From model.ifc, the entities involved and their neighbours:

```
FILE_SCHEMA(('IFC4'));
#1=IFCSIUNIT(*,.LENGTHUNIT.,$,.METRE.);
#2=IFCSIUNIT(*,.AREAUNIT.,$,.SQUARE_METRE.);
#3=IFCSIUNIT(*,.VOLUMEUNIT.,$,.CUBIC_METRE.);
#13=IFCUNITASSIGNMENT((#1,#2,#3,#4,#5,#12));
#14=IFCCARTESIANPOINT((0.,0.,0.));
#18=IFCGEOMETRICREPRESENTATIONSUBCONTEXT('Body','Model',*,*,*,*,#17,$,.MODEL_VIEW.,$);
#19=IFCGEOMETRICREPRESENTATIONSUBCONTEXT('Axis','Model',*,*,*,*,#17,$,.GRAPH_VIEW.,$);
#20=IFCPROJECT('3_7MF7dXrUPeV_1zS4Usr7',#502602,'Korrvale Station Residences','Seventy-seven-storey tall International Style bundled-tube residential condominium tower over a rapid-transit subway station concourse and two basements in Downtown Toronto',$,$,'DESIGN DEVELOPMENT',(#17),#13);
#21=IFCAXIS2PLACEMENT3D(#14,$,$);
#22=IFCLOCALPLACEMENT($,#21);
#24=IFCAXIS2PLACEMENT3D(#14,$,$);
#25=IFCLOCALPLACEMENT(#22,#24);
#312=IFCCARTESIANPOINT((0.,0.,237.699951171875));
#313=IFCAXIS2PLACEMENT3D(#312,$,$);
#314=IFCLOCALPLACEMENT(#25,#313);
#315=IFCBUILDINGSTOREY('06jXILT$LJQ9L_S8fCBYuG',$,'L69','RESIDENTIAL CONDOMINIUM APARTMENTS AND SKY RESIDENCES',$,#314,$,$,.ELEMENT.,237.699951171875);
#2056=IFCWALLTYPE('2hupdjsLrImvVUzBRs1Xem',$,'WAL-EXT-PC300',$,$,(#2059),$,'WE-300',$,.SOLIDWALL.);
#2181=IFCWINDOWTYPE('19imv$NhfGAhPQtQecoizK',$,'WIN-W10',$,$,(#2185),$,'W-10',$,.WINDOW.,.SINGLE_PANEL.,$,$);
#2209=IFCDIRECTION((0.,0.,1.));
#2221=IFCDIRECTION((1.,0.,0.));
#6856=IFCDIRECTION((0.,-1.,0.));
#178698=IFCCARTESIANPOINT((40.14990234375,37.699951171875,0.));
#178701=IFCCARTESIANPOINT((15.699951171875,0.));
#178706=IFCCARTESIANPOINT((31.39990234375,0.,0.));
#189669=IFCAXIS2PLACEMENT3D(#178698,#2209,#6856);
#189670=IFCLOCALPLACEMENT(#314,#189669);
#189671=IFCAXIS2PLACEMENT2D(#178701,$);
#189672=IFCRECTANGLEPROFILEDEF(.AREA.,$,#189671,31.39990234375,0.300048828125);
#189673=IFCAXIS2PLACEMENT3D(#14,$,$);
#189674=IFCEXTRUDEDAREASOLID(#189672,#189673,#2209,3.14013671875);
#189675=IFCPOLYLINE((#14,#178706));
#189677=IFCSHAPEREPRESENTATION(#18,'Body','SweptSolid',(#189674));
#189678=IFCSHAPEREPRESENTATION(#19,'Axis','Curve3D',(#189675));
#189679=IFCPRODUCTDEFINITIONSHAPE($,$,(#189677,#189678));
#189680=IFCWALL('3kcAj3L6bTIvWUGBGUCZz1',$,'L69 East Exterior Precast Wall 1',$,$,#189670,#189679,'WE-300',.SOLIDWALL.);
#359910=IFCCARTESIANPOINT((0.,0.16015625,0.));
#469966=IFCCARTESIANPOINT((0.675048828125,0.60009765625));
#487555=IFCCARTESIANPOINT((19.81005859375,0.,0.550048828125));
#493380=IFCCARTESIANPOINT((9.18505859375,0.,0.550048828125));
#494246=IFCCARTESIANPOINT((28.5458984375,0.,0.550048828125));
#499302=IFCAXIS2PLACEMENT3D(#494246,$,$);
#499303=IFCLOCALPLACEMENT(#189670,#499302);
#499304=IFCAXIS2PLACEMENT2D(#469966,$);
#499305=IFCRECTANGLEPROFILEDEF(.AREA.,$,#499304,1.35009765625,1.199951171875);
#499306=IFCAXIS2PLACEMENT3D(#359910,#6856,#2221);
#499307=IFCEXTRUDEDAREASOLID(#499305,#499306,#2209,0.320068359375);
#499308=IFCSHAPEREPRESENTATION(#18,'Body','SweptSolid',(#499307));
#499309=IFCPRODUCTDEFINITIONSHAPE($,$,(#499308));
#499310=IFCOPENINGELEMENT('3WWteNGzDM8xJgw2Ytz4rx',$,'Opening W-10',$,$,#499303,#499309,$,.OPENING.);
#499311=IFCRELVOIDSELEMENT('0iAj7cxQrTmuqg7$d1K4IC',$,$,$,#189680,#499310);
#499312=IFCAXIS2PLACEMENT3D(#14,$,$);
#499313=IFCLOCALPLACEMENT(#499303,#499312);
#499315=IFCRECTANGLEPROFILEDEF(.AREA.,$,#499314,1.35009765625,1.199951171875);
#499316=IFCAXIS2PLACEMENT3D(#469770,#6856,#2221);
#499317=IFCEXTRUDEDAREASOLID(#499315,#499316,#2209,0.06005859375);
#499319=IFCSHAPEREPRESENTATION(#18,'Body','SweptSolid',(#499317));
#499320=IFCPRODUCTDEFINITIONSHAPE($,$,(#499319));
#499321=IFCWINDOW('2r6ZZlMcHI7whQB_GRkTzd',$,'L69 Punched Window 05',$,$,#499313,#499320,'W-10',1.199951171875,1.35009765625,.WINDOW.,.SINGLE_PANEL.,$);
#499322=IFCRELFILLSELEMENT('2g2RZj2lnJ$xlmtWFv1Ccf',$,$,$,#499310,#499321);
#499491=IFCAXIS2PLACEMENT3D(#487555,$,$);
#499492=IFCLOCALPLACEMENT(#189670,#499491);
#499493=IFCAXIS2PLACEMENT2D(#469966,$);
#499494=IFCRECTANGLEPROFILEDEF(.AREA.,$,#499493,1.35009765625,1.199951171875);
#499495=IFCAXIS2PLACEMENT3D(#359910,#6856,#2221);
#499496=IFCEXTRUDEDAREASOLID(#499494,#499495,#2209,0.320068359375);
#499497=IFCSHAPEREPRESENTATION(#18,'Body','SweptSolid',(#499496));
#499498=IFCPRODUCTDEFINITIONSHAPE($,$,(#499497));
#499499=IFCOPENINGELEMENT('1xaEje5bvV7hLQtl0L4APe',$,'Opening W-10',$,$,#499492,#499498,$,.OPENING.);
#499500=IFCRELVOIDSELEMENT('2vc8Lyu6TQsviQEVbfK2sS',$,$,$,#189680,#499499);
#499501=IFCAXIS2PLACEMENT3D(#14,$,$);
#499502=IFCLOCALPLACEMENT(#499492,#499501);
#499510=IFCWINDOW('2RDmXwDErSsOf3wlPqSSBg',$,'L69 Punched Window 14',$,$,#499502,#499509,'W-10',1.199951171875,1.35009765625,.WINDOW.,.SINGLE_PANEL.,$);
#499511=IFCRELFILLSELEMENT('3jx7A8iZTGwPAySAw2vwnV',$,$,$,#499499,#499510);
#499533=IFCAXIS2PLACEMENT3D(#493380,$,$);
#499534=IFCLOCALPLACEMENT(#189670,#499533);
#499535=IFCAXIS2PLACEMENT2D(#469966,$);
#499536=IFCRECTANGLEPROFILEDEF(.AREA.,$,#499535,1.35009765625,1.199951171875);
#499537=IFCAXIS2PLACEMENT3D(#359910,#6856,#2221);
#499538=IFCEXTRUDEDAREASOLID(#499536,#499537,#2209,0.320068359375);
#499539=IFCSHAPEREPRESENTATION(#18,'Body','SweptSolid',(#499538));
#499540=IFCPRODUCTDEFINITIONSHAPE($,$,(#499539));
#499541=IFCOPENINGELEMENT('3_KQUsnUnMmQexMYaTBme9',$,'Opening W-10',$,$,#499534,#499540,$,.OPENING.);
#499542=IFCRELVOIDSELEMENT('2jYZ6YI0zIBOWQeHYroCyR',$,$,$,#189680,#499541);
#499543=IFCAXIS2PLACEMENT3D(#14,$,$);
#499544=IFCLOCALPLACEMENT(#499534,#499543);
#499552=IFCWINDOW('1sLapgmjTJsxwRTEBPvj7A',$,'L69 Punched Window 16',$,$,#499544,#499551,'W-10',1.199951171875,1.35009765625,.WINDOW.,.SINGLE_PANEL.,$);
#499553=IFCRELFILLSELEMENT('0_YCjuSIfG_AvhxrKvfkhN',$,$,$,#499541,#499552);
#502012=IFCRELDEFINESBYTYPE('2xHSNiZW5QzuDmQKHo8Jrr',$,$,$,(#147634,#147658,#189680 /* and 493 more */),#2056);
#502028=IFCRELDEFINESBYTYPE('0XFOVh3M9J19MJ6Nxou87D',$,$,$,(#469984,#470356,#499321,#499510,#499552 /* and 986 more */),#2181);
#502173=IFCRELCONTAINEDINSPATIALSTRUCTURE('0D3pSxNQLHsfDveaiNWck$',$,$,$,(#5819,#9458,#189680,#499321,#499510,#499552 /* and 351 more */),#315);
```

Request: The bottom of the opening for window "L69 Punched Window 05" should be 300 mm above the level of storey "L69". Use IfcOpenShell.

```python
import numpy as np
import ifcopenshell
import ifcopenshell.api.geometry
import ifcopenshell.geom
import ifcopenshell.util.element
import ifcopenshell.util.placement
import ifcopenshell.util.shape
import ifcopenshell.util.unit

model = ifcopenshell.open("model.ifc")
unit_scale = ifcopenshell.util.unit.calculate_unit_scale(model)

window = model.by_guid("2r6ZZlMcHI7whQB_GRkTzd")
opening = window.FillsVoids[0].RelatingOpeningElement
storey = ifcopenshell.util.element.get_container(window, ifc_class="IfcBuildingStorey")
level = ifcopenshell.util.placement.get_local_placement(storey.ObjectPlacement)[2, 3]

# The opening's origin need not be at the sill, so measure its lowest point.
shape = ifcopenshell.geom.create_shape(ifcopenshell.geom.settings(), opening)
bottom = ifcopenshell.util.shape.get_shape_bottom_elevation(shape, shape.geometry) / unit_scale
dz = level + 0.3 - bottom

shift = np.array([0.0, 0.0, dz])
# The window is placed relative to its opening, so it follows when the opening moves.
matrix = ifcopenshell.util.placement.get_local_placement(opening.ObjectPlacement)
matrix[:3, 3] += shift
ifcopenshell.api.geometry.edit_object_placement(
    model, product=opening, matrix=matrix, is_si=False, should_transform_children=True
)

print(f"moved by {dz * unit_scale:+.3f} m")

model.write("model_v2.ifc")
```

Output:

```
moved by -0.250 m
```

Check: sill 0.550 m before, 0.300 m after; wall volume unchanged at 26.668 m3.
